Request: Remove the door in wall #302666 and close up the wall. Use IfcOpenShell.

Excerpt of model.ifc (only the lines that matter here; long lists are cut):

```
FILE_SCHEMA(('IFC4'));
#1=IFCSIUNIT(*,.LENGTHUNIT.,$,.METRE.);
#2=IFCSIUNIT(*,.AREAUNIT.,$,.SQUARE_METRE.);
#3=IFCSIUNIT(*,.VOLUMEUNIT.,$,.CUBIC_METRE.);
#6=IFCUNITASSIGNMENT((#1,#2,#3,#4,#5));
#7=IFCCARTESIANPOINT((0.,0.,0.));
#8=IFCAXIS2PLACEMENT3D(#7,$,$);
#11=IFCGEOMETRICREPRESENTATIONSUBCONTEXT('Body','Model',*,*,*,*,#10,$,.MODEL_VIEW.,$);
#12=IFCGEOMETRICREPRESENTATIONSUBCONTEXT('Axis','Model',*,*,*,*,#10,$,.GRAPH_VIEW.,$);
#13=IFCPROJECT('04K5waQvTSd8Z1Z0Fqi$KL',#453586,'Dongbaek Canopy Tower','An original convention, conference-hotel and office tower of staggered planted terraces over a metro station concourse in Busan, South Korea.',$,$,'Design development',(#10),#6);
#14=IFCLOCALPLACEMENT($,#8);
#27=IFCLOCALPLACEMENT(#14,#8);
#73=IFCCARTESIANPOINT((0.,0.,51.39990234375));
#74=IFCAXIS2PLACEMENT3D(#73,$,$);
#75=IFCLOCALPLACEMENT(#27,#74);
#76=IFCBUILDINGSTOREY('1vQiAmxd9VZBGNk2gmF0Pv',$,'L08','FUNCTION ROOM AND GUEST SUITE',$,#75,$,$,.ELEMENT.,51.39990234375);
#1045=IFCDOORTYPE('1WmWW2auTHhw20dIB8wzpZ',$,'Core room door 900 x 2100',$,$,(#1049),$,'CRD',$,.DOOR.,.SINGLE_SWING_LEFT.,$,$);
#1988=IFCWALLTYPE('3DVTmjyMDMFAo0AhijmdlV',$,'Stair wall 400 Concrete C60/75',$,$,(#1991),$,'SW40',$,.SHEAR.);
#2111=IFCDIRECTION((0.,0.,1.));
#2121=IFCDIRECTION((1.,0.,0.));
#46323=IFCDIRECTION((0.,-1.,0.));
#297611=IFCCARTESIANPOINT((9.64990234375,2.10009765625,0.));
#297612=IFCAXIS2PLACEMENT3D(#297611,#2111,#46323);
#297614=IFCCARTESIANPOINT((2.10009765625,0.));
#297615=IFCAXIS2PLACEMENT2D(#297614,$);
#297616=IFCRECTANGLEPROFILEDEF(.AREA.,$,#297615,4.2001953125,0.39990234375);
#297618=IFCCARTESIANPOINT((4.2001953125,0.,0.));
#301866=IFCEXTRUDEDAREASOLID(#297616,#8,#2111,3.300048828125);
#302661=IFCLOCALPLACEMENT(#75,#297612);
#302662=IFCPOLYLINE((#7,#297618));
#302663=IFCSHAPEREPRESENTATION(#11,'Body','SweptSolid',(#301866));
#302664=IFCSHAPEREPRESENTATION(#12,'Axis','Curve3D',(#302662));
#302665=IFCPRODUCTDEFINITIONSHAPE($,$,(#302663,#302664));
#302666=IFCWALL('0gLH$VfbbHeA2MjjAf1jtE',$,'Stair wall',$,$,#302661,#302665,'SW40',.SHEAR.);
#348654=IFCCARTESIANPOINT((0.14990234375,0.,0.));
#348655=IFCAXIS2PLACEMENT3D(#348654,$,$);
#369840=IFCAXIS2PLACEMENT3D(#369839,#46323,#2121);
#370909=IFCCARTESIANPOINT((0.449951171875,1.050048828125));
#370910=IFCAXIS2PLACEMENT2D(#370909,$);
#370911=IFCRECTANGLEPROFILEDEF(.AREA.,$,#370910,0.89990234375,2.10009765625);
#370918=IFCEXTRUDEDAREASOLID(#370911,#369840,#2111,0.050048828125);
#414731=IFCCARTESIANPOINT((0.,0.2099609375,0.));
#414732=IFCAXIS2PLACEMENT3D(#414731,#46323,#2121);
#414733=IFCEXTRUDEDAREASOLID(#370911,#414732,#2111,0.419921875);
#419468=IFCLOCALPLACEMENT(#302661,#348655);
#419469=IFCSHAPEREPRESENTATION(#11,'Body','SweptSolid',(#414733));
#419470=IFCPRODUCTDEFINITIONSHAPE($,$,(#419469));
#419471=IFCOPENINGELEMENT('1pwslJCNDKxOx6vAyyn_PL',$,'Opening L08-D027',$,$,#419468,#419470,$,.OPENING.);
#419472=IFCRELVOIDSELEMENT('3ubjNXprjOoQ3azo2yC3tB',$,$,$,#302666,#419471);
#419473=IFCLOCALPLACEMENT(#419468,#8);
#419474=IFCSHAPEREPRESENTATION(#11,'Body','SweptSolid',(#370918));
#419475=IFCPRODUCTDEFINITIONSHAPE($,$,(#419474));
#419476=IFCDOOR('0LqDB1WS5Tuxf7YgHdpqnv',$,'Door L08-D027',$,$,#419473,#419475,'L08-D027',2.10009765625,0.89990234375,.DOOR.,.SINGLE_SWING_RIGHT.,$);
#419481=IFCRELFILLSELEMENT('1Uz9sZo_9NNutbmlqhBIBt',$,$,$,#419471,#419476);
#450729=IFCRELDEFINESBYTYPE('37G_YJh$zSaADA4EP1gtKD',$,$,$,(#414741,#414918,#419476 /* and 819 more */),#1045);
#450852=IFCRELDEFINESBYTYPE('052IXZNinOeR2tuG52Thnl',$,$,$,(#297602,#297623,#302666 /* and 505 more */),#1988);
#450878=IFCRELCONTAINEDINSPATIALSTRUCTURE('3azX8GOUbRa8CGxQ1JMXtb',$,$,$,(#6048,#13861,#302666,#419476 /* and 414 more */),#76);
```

```python
import ifcopenshell
import ifcopenshell.api.feature
import ifcopenshell.api.root
import ifcopenshell.geom
import ifcopenshell.util.shape

model = ifcopenshell.open("model.ifc")
settings = ifcopenshell.geom.settings()


def volume(element):
    """Net volume in cubic metres, openings subtracted."""
    shape = ifcopenshell.geom.create_shape(settings, element)
    return ifcopenshell.util.shape.get_volume(shape.geometry)


door = model.by_guid("0LqDB1WS5Tuxf7YgHdpqnv")
opening = door.FillsVoids[0].RelatingOpeningElement
wall = opening.VoidsElements[0].RelatingBuildingElement
before = volume(wall)

ifcopenshell.api.root.remove_product(model, product=door)
ifcopenshell.api.feature.remove_feature(model, feature=opening)

after = volume(wall)

print(f"wall volume {before:.3f} -> {after:.3f} m3")

model.write("model_updated.ifc")
```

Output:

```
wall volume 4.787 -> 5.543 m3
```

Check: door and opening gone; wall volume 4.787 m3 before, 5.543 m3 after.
